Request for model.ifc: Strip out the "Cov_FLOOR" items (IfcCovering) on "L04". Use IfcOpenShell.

First a look at what the model holds.

```python
import ifcopenshell
import ifcopenshell.util.element

model = ifcopenshell.open("model.ifc")
print(model.schema)
storey = next(s for s in model.by_type("IfcBuildingStorey") if s.Name == "L04")
coverings = [e for e in ifcopenshell.util.element.get_decomposition(storey) if e.is_a("IfcCovering")]
seen = {}
for e in coverings:
    element_type = ifcopenshell.util.element.get_type(e)
    name = element_type.Name if element_type not in (None, e) else None
    seen[name] = seen.get(name, 0) + 1
for name, count in sorted(seen.items(), key=str):
    print(count, "x", name)
```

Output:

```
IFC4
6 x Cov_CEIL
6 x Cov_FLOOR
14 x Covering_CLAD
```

```python
import ifcopenshell
import ifcopenshell.api.root
import ifcopenshell.util.element

model = ifcopenshell.open("model.ifc")

storey = next(s for s in model.by_type("IfcBuildingStorey") if s.Name == "L04")
coverings = [e for e in ifcopenshell.util.element.get_decomposition(storey) if e.is_a("IfcCovering")]
targets = [e for e in coverings if (t := ifcopenshell.util.element.get_type(e)) not in (None, e) and t.Name == "Cov_FLOOR"]

for e in targets:
    ifcopenshell.api.root.remove_product(model, product=e)
print(len(targets), "removed")

model.write("model_v2.ifc")
```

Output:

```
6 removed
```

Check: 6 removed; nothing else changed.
